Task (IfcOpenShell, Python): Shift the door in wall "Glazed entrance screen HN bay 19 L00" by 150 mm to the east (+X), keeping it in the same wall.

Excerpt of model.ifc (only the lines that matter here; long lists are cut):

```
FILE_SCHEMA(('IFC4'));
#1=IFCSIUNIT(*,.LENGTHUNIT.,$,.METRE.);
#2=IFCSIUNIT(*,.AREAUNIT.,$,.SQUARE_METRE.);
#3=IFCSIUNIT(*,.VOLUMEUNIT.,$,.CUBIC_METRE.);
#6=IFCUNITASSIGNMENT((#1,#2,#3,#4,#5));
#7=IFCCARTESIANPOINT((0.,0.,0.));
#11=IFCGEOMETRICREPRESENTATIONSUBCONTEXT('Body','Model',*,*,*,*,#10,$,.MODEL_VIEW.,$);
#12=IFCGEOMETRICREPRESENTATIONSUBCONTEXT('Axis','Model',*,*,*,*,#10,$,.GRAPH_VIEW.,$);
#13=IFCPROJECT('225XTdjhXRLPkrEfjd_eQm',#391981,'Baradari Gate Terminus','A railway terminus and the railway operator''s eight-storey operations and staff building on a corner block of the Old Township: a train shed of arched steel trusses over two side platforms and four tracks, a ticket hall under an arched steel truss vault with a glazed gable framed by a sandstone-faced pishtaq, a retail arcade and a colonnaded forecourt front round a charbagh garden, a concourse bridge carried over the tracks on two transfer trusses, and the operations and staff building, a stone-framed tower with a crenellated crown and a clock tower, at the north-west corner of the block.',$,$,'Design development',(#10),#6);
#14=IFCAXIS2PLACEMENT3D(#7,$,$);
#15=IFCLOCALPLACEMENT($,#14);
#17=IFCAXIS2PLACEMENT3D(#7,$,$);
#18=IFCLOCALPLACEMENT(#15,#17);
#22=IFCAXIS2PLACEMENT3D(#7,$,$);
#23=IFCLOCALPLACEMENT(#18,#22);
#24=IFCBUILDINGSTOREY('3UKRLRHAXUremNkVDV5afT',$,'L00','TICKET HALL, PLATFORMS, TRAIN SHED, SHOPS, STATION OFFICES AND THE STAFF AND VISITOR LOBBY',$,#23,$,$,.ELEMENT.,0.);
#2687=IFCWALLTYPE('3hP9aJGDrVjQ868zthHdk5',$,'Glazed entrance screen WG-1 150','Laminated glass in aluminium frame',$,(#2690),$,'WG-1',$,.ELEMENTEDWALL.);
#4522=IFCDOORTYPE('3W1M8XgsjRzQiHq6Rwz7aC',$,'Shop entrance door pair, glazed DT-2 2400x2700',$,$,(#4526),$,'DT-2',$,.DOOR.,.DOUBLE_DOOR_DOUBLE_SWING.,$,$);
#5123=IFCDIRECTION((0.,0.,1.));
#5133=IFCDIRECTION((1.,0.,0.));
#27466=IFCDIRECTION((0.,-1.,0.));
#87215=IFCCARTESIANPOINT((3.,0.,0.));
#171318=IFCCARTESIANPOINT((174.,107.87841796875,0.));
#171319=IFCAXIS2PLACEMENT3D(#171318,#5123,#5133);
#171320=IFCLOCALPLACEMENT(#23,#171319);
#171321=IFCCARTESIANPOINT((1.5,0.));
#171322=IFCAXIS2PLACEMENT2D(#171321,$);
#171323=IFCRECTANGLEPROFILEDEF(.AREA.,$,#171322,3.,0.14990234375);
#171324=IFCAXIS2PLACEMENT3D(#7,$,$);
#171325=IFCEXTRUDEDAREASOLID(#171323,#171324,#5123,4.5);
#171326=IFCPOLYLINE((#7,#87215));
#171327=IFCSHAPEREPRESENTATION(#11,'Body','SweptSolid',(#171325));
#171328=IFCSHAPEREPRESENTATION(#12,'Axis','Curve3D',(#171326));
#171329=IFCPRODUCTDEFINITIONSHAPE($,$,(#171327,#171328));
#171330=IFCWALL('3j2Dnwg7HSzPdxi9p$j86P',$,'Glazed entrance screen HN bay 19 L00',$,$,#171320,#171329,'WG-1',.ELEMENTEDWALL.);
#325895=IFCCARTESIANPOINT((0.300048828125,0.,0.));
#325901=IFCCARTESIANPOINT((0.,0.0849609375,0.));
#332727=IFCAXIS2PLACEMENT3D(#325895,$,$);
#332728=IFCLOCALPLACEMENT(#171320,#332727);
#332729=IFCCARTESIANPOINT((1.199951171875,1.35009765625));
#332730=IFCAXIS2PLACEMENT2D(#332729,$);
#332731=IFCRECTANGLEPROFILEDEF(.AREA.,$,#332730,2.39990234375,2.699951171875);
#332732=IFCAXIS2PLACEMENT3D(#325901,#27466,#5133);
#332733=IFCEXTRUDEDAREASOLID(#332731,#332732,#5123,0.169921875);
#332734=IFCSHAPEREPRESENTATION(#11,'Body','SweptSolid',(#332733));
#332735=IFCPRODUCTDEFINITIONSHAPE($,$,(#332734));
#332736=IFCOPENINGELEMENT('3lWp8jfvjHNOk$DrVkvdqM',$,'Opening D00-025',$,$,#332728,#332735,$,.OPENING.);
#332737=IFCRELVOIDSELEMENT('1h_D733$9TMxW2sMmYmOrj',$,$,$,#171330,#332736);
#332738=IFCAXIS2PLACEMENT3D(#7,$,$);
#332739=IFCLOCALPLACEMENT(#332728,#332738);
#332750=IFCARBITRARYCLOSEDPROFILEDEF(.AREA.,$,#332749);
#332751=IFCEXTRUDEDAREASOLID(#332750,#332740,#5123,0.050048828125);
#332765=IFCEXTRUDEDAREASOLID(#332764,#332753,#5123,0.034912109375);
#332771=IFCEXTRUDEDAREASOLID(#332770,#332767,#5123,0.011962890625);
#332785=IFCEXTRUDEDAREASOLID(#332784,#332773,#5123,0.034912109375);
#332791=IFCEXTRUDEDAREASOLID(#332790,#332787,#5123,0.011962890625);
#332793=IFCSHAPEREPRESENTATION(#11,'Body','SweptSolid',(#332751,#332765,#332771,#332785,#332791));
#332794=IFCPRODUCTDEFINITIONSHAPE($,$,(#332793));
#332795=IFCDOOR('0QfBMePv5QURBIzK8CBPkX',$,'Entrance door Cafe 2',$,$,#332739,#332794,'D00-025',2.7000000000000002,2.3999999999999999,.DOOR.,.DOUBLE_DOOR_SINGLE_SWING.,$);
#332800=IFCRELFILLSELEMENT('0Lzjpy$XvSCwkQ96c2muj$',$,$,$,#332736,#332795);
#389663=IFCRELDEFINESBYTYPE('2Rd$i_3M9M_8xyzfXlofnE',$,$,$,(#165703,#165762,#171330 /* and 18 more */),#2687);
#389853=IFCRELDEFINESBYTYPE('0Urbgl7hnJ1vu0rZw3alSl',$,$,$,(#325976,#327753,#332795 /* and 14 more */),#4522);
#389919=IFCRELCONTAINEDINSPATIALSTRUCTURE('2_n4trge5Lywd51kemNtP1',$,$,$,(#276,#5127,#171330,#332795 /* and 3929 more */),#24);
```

```python
import ifcopenshell
import ifcopenshell.api.geometry
import ifcopenshell.util.placement

model = ifcopenshell.open("model.ifc")

door = model.by_id(332795)
opening = door.FillsVoids[0].RelatingOpeningElement
wall = opening.VoidsElements[0].RelatingBuildingElement

wall_matrix = ifcopenshell.util.placement.get_local_placement(wall.ObjectPlacement)
shift = wall_matrix[:3, 0] * 0.15
before = ifcopenshell.util.placement.get_local_placement(door.ObjectPlacement)[:3, 3].copy()

# The door is placed relative to its opening, so it follows when the opening moves.
matrix = ifcopenshell.util.placement.get_local_placement(opening.ObjectPlacement)
matrix[:3, 3] += shift
ifcopenshell.api.geometry.edit_object_placement(
    model, product=opening, matrix=matrix, is_si=False, should_transform_children=True
)

after = ifcopenshell.util.placement.get_local_placement(door.ObjectPlacement)[:3, 3]
print("door moved by", (after - before).round(3) + 0.0)

model.write("model_v2.ifc")
```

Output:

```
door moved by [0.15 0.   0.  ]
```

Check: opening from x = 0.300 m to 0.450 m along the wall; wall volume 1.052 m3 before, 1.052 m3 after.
